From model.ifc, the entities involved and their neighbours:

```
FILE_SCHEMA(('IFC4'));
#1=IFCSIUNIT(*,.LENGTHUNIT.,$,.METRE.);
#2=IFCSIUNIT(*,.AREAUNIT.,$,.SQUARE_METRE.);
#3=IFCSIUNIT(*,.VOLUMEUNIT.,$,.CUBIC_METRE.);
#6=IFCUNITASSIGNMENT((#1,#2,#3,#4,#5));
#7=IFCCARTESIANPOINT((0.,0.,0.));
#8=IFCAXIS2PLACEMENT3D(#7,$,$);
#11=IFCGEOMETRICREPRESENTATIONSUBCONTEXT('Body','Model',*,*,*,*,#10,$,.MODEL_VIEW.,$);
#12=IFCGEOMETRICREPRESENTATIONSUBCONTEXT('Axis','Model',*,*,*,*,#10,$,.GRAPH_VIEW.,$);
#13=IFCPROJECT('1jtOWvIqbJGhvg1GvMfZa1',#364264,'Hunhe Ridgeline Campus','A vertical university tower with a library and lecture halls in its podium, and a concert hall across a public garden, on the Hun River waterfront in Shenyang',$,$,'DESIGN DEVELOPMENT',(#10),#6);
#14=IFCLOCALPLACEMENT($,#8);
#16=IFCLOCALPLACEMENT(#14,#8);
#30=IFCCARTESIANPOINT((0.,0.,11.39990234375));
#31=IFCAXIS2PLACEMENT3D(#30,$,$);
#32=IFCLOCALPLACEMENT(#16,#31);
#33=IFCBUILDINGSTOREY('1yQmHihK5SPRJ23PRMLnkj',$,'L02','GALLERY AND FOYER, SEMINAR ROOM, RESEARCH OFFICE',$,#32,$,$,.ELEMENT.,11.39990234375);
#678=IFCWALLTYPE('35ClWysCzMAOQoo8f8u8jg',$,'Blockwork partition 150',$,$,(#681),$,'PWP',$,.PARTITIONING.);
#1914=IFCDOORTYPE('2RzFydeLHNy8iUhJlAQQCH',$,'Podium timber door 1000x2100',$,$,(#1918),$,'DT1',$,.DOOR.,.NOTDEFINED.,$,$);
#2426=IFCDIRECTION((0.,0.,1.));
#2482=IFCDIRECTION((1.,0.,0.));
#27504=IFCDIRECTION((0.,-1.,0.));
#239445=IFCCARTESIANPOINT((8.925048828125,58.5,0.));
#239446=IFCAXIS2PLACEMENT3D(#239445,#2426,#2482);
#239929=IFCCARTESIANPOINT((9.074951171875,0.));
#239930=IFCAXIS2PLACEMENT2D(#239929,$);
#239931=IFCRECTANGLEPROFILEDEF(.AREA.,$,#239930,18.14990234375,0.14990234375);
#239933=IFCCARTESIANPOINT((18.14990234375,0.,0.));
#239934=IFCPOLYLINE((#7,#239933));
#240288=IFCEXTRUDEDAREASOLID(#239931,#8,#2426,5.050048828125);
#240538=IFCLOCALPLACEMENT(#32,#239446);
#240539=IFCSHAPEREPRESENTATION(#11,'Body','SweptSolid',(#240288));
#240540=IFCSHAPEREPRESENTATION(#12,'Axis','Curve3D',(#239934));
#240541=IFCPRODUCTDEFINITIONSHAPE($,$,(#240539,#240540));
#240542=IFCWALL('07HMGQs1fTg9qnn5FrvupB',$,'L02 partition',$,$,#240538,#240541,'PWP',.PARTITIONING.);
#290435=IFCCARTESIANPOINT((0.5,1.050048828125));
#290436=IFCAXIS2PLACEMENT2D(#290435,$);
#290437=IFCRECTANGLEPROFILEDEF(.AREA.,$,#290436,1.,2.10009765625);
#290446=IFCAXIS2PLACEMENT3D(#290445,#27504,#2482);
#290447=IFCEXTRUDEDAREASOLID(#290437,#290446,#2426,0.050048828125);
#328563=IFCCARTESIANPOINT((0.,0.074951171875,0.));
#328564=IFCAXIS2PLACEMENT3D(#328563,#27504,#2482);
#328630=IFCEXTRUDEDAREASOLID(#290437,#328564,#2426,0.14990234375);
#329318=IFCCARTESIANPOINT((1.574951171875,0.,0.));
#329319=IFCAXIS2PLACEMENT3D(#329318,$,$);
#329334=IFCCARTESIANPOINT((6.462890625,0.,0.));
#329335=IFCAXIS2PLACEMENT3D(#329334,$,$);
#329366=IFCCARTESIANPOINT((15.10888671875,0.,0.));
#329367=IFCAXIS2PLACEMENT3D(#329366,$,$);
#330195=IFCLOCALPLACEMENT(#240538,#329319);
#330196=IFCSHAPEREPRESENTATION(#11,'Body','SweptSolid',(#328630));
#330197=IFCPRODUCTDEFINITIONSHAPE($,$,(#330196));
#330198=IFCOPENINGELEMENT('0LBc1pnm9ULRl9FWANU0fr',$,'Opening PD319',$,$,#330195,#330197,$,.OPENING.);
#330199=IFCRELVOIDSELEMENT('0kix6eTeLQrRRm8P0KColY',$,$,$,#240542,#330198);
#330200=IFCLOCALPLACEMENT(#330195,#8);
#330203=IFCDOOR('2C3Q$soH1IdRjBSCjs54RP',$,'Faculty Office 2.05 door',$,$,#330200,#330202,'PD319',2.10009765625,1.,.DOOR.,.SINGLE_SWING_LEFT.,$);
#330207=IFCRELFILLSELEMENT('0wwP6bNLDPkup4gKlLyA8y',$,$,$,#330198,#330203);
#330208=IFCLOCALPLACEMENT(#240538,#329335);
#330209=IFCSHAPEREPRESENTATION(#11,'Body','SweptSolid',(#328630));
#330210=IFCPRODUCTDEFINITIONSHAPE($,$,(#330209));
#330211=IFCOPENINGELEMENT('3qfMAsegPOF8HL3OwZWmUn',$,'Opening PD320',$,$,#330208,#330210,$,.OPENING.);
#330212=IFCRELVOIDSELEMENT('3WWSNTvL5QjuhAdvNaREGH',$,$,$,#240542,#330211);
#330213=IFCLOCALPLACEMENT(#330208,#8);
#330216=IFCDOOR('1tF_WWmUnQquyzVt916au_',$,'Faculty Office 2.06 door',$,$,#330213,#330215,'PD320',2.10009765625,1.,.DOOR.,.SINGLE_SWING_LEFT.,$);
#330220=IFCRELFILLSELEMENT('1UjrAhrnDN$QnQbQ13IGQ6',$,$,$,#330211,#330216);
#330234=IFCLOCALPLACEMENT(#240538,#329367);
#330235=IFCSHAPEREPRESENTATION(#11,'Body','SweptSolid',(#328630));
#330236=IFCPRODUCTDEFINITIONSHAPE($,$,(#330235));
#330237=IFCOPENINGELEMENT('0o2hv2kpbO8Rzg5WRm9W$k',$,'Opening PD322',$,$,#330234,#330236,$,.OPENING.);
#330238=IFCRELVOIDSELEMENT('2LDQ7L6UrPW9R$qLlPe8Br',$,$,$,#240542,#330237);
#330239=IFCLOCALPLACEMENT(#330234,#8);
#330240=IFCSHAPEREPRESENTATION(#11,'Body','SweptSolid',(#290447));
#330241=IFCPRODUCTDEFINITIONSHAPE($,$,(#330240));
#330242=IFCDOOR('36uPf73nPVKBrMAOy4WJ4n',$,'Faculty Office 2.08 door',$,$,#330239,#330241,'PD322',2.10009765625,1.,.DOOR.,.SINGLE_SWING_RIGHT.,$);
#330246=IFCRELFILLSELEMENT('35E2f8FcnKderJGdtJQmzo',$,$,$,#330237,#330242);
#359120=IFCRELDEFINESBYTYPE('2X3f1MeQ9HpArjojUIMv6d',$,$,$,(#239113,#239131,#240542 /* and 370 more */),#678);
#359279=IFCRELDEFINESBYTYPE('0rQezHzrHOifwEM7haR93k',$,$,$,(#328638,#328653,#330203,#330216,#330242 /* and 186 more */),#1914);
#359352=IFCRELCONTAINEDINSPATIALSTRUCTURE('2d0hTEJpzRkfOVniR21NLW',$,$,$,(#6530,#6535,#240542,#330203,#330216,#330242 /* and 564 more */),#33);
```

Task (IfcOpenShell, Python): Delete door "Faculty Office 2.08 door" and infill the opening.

```python
import ifcopenshell
import ifcopenshell.api.feature
import ifcopenshell.api.root
import ifcopenshell.geom
import ifcopenshell.util.shape

model = ifcopenshell.open("model.ifc")
settings = ifcopenshell.geom.settings()


def volume(element):
    """Net volume in cubic metres, openings subtracted."""
    shape = ifcopenshell.geom.create_shape(settings, element)
    return ifcopenshell.util.shape.get_volume(shape.geometry)


door = model.by_guid("36uPf73nPVKBrMAOy4WJ4n")
opening = door.FillsVoids[0].RelatingOpeningElement
wall = opening.VoidsElements[0].RelatingBuildingElement
before = volume(wall)

ifcopenshell.api.root.remove_product(model, product=door)
ifcopenshell.api.feature.remove_feature(model, feature=opening)

after = volume(wall)

print(f"wall volume {before:.3f} -> {after:.3f} m3")

model.write("model_rev.ifc")
```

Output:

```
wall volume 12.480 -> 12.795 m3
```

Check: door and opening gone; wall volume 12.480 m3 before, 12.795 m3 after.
